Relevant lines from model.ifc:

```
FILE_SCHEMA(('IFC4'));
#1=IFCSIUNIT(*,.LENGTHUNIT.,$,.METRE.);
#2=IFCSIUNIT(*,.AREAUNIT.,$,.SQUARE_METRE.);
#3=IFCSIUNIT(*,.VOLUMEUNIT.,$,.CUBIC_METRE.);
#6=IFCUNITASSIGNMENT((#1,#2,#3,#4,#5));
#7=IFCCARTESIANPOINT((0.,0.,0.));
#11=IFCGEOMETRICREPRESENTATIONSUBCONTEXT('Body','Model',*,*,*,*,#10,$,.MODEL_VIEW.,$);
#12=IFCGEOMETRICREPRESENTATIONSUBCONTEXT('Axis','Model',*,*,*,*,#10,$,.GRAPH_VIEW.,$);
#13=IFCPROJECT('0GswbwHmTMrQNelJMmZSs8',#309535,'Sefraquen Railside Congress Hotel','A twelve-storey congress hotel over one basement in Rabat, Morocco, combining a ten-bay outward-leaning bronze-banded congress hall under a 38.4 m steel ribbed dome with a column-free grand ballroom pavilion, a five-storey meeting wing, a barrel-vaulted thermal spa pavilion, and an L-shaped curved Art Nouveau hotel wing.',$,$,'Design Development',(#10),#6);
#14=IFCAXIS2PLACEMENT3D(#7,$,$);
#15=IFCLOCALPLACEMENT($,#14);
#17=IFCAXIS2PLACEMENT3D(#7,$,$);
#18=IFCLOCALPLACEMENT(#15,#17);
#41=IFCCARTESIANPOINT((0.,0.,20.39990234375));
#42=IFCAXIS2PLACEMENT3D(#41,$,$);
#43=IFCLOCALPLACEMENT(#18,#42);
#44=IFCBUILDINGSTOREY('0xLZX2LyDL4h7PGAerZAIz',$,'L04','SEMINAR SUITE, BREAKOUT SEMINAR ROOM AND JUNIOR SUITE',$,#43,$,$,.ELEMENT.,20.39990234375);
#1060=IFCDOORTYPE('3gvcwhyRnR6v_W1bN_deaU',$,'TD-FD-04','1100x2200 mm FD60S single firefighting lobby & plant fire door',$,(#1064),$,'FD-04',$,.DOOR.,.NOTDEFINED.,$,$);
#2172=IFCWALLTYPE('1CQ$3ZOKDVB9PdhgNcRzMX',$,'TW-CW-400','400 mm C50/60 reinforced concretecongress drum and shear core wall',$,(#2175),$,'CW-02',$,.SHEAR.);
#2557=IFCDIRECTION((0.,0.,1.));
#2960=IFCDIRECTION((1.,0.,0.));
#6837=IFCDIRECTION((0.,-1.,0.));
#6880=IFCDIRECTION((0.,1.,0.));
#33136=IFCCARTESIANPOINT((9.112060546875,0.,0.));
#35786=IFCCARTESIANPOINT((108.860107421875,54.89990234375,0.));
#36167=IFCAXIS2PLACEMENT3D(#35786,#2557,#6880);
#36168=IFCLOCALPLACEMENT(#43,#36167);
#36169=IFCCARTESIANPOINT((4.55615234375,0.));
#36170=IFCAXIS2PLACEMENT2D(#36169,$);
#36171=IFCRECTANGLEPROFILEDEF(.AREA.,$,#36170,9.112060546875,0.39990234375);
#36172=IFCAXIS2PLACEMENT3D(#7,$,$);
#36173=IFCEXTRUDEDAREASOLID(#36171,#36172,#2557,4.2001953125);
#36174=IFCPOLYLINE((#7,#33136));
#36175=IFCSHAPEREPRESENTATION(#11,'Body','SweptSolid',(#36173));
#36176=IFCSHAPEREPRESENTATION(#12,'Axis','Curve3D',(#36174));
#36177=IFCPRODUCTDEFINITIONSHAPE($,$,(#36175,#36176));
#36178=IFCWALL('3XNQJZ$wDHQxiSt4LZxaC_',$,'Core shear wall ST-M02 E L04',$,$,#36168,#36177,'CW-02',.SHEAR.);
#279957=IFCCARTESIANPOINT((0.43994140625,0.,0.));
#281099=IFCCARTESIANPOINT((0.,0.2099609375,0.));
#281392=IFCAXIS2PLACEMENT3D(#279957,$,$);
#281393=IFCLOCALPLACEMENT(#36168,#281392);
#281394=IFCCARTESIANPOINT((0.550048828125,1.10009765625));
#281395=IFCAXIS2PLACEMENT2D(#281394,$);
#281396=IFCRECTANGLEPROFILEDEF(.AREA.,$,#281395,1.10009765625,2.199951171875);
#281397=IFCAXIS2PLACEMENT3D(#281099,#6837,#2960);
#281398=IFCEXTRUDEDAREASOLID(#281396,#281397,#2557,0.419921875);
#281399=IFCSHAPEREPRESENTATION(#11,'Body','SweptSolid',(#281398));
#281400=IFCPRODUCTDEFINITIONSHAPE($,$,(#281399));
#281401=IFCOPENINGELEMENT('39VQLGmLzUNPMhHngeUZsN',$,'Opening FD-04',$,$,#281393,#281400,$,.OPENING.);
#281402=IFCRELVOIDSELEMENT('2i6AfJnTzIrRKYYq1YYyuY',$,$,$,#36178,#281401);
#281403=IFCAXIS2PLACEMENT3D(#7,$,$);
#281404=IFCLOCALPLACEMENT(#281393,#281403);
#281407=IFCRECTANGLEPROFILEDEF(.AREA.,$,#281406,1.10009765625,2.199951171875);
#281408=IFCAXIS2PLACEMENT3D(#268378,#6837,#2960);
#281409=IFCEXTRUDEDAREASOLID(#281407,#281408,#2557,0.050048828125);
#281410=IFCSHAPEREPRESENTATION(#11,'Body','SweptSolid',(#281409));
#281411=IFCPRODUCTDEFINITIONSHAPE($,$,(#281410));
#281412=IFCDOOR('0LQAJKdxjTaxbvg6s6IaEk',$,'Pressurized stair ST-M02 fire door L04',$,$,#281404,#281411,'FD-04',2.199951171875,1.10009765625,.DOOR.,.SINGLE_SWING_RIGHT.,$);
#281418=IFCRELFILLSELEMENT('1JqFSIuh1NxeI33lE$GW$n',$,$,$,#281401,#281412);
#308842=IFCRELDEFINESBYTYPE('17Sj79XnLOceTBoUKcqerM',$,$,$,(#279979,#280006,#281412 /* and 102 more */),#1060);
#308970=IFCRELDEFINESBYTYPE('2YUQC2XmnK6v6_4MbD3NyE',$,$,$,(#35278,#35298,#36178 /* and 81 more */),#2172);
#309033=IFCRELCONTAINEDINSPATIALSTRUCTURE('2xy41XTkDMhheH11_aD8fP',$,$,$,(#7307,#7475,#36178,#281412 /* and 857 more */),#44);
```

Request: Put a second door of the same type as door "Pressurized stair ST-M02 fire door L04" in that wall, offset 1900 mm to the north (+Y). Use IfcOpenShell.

```python
import ifcopenshell
import ifcopenshell.api.feature
import ifcopenshell.api.geometry
import ifcopenshell.api.root
import ifcopenshell.geom
import ifcopenshell.util.element
import ifcopenshell.util.placement
import ifcopenshell.util.shape

model = ifcopenshell.open("model.ifc")
settings = ifcopenshell.geom.settings()


def volume(element):
    """Net volume in cubic metres, openings subtracted."""
    shape = ifcopenshell.geom.create_shape(settings, element)
    return ifcopenshell.util.shape.get_volume(shape.geometry)


door = model.by_id(281412)
opening = door.FillsVoids[0].RelatingOpeningElement
wall = opening.VoidsElements[0].RelatingBuildingElement
before = volume(wall)
shift = ifcopenshell.util.placement.get_local_placement(wall.ObjectPlacement)[:3, 0] * 1.9

# copy_class copies the void relationship, type, container and properties, but no geometry.
new_opening = ifcopenshell.api.root.copy_class(model, product=opening)
new_opening.Representation = ifcopenshell.util.element.copy_deep(
    model, opening.Representation, exclude=["IfcGeometricRepresentationContext", "IfcRepresentationMap"]
)
new_door = ifcopenshell.api.root.copy_class(model, product=door)
new_door.Representation = ifcopenshell.util.element.copy_deep(
    model, door.Representation, exclude=["IfcGeometricRepresentationContext", "IfcRepresentationMap"]
)
new_door.Tag = None
ifcopenshell.api.feature.add_filling(model, opening=new_opening, element=new_door)

for old, new in ((opening, new_opening), (door, new_door)):
    matrix = ifcopenshell.util.placement.get_local_placement(old.ObjectPlacement)
    matrix[:3, 3] += shift
    ifcopenshell.api.geometry.edit_object_placement(model, product=new, matrix=matrix, is_si=False)

after = volume(wall)

print(f"wall volume {before:.3f} -> {after:.3f} m3")

model.write("model_rev.ifc")
```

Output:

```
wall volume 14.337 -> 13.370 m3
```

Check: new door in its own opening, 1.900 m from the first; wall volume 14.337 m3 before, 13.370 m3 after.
